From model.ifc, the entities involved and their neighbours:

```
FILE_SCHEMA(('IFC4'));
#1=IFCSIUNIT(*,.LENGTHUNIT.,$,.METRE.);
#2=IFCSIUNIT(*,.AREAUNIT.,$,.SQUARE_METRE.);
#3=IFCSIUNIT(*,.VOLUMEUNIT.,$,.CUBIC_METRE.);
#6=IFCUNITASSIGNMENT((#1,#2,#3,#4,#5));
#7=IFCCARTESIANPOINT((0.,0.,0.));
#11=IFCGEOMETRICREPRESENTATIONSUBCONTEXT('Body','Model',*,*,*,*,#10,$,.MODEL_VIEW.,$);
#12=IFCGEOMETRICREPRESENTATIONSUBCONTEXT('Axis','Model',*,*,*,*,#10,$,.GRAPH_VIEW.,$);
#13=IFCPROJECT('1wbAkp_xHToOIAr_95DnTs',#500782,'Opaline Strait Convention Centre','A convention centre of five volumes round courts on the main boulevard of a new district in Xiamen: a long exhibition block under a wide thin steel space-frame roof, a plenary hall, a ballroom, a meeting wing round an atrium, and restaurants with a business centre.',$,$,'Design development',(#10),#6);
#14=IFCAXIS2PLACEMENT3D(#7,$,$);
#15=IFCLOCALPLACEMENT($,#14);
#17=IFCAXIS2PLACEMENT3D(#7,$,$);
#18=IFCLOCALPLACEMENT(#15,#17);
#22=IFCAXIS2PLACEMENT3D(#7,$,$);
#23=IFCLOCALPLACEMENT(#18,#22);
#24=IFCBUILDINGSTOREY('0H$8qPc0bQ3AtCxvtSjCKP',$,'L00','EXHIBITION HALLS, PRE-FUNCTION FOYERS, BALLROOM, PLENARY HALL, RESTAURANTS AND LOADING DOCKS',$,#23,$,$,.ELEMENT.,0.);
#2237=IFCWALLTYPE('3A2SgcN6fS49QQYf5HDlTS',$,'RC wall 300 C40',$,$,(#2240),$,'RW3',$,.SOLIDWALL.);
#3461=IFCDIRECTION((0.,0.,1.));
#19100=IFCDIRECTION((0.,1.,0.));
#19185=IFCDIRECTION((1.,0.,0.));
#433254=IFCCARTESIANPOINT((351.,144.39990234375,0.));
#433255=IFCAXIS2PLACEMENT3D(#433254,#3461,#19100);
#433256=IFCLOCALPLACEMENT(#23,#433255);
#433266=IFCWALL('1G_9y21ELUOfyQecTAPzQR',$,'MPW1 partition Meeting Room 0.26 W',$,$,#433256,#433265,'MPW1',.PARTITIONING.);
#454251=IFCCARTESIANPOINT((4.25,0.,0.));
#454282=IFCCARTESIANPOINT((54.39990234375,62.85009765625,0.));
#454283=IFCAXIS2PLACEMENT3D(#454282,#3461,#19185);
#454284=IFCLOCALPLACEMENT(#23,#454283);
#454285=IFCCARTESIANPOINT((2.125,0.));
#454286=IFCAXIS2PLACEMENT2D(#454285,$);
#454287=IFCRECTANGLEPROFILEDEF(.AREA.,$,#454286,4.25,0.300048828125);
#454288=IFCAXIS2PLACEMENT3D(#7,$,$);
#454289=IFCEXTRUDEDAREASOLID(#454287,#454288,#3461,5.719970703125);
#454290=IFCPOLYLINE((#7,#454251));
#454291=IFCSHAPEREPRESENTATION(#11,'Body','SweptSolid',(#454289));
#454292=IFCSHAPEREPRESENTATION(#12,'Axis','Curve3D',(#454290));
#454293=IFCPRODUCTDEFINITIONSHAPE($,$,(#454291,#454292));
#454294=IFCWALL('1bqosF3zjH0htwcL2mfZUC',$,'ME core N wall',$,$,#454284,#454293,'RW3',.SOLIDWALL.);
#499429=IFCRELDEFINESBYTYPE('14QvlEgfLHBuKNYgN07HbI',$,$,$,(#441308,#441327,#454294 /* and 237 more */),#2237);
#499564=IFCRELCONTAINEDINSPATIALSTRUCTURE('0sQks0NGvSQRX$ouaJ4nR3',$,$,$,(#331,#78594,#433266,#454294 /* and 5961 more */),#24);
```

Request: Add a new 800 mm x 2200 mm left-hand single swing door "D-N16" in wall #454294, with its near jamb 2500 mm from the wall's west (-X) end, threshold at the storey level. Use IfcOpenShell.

```python
import numpy as np
import ifcopenshell
import ifcopenshell.api.feature
import ifcopenshell.api.geometry
import ifcopenshell.api.root
import ifcopenshell.api.spatial
import ifcopenshell.geom
import ifcopenshell.util.element
import ifcopenshell.util.placement
import ifcopenshell.util.representation
import ifcopenshell.util.shape
import ifcopenshell.util.unit

model = ifcopenshell.open("model.ifc")
unit_scale = ifcopenshell.util.unit.calculate_unit_scale(model)
settings = ifcopenshell.geom.settings()


def volume(element):
    """Net volume in cubic metres, openings subtracted."""
    shape = ifcopenshell.geom.create_shape(settings, element)
    return ifcopenshell.util.shape.get_volume(shape.geometry)


wall = model.by_guid("1bqosF3zjH0htwcL2mfZUC")
storey = ifcopenshell.util.element.get_container(wall, ifc_class="IfcBuildingStorey")
context = ifcopenshell.util.representation.get_context(model, "Model", "Body", "MODEL_VIEW")
before = volume(wall)

width, height, from_end, sill = 0.8, 2.2, 2.5, 0.0  # metres

# The wall runs along its own X axis, and the end named is its -X end.
wall_shape = ifcopenshell.geom.create_shape(settings, wall)
x, y, z = ifcopenshell.util.shape.get_vertices(wall_shape.geometry).T
start = x.min() + from_end
face, thickness = float(y.min()), float(y.max() - y.min())
wall_matrix = ifcopenshell.util.placement.get_local_placement(wall.ObjectPlacement)
level = ifcopenshell.util.placement.get_local_placement(storey.ObjectPlacement)[2, 3]


def in_wall(x, y):
    """Placement at x, y metres in the wall's axes, at sill height."""
    matrix = wall_matrix.copy()
    matrix[:, 3] = wall_matrix @ np.array([x / unit_scale, y / unit_scale, 0.0, 1.0])
    matrix[2, 3] = level + sill / unit_scale
    return matrix


# Opening: a box that overshoots both wall faces by 50 mm.
opening = ifcopenshell.api.root.create_entity(model, ifc_class="IfcOpeningElement", predefined_type="OPENING")
box = ifcopenshell.api.geometry.add_wall_representation(
    model, context=context, length=width, height=height, thickness=thickness + 0.1
)
ifcopenshell.api.geometry.assign_representation(model, product=opening, representation=box)
ifcopenshell.api.geometry.edit_object_placement(model, product=opening, matrix=in_wall(start, face - 0.05), is_si=False)
ifcopenshell.api.feature.add_feature(model, feature=opening, element=wall)

door = ifcopenshell.api.root.create_entity(model, ifc_class="IfcDoor", name="D-N16", predefined_type="DOOR")
door.OverallWidth, door.OverallHeight = width / unit_scale, height / unit_scale
door.OperationType = "SINGLE_SWING_LEFT"
body = ifcopenshell.api.geometry.add_door_representation(
    model,
    context=context,
    overall_width=door.OverallWidth,
    overall_height=door.OverallHeight,
    operation_type="SINGLE_SWING_LEFT",
    lining_properties={"LiningDepth": thickness / unit_scale, "ThresholdDepth": thickness / unit_scale},
)
ifcopenshell.api.geometry.assign_representation(model, product=door, representation=body)
ifcopenshell.api.spatial.assign_container(model, products=[door], relating_structure=storey)
ifcopenshell.api.feature.add_filling(model, opening=opening, element=door)

# The lining spans the wall, so the door starts at the wall face.
ifcopenshell.api.geometry.edit_object_placement(model, product=door, matrix=in_wall(start, face), is_si=False)

after = volume(wall)

print(f"wall volume {before:.3f} -> {after:.3f} m3")

model.write("model_updated.ifc")
```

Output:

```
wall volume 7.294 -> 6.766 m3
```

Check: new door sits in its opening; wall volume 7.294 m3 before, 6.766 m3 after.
